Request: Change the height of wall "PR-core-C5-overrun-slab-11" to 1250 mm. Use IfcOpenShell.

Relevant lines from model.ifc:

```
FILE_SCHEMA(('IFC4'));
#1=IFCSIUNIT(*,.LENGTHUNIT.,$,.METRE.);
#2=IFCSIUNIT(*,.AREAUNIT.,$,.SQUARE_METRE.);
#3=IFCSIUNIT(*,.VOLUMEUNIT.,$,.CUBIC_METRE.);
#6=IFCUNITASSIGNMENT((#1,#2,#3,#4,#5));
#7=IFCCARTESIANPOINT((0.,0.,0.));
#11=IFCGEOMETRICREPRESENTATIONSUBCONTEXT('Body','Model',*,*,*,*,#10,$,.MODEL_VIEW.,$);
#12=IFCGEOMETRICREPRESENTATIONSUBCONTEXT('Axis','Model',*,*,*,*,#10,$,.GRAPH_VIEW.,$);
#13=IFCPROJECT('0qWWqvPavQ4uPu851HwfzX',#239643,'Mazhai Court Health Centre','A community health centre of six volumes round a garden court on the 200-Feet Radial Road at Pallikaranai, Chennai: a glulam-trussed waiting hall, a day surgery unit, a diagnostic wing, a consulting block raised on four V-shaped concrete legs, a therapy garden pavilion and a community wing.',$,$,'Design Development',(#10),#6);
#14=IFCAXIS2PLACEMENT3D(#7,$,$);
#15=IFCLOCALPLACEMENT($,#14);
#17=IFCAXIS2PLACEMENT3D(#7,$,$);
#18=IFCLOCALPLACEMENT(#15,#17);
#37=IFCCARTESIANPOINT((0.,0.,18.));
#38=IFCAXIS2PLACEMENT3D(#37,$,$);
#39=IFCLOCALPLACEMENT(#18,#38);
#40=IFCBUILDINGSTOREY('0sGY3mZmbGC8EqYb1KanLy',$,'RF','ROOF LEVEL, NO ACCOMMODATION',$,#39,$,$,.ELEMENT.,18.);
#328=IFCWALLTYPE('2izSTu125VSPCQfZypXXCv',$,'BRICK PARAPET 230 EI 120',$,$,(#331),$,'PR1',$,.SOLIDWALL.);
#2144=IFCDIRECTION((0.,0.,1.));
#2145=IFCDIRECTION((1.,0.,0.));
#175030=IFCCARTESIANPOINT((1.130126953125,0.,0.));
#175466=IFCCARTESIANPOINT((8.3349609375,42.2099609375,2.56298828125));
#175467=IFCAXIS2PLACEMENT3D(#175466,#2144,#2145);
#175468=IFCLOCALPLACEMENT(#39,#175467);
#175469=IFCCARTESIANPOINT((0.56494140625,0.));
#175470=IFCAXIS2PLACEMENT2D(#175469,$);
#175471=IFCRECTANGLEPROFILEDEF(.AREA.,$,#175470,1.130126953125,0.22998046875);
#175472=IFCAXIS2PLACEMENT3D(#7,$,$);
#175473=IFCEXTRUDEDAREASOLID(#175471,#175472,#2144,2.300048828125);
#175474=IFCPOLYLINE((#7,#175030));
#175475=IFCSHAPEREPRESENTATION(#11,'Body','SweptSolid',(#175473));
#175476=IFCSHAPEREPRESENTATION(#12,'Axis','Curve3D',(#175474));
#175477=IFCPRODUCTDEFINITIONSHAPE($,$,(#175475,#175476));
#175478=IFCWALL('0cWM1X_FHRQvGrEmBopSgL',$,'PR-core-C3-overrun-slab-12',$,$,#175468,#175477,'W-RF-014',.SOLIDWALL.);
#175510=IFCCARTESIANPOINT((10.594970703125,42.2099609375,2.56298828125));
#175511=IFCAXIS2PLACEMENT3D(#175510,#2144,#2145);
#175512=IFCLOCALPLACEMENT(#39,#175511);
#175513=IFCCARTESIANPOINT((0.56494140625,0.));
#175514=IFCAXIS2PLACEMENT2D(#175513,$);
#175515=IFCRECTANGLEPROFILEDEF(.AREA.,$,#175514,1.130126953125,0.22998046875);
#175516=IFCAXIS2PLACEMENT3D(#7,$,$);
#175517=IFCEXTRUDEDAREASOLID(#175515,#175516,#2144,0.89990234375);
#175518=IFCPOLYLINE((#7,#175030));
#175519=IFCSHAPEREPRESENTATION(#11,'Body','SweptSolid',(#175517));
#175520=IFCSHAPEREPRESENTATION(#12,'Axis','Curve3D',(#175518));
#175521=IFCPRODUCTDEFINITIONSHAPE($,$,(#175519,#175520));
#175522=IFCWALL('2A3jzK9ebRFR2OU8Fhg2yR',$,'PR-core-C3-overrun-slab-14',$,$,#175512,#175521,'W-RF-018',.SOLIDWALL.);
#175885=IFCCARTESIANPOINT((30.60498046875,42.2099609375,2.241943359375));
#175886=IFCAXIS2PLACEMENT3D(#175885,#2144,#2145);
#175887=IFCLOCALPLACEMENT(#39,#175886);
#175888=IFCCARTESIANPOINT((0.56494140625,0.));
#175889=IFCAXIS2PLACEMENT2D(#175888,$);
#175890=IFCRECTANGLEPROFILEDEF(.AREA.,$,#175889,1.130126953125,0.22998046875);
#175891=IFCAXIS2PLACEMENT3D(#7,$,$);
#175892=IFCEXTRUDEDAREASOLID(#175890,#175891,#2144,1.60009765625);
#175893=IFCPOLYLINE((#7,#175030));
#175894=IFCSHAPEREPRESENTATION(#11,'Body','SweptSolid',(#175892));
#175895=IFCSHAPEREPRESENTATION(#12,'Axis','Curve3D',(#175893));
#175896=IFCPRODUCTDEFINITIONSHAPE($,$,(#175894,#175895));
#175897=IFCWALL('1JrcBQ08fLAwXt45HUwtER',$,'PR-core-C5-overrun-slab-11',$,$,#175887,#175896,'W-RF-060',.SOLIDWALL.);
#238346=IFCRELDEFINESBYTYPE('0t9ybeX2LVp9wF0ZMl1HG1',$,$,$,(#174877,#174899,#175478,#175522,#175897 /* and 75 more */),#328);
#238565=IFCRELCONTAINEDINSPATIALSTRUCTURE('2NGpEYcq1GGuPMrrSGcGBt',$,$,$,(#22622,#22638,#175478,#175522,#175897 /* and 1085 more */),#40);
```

```python
import ifcopenshell
import ifcopenshell.geom
import ifcopenshell.util.representation
import ifcopenshell.util.shape

model = ifcopenshell.open("model.ifc")
settings = ifcopenshell.geom.settings()


def volume(element):
    """Net volume in cubic metres, openings subtracted."""
    shape = ifcopenshell.geom.create_shape(settings, element)
    return ifcopenshell.util.shape.get_volume(shape.geometry)


wall = model.by_id(175897)
before = volume(wall)

body = ifcopenshell.util.representation.get_representation(wall, "Model", "Body")
solid = body.Items[0]
old_height = solid.Depth
solid.Depth = 1.25
after = volume(wall)

print(f"height {old_height:g} -> {solid.Depth:g}, volume {before:.3f} -> {after:.3f} m3")

model.write("model_v2.ifc")
```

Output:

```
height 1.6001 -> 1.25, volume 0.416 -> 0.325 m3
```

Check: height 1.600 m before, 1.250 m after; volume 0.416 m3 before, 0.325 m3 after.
